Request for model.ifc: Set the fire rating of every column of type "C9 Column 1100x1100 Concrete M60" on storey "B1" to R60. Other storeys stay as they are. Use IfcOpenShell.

First a look at what the model holds.

```python
import ifcopenshell
import ifcopenshell.util.element

model = ifcopenshell.open("model.ifc")
print(model.schema)
storey = next(s for s in model.by_type("IfcBuildingStorey") if s.Name == "B1")
columns = [e for e in ifcopenshell.util.element.get_decomposition(storey) if e.is_a("IfcColumn")]
seen = {}
for e in columns:
    element_type = ifcopenshell.util.element.get_type(e)
    key = (element_type.Name if element_type != e and element_type else None, ifcopenshell.util.element.get_pset(e, "Pset_ColumnCommon", "FireRating"))
    seen[key] = seen.get(key, 0) + 1
for (name, value), count in sorted(seen.items(), key=str):
    print(count, "x", name, "|", value)
```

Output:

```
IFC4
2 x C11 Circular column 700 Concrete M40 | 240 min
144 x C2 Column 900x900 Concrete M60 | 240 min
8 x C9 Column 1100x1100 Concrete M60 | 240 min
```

```python
import ifcopenshell
import ifcopenshell.api.pset
import ifcopenshell.util.element

model = ifcopenshell.open("model.ifc")

storey = next(s for s in model.by_type("IfcBuildingStorey") if s.Name == "B1")
columns = [e for e in ifcopenshell.util.element.get_decomposition(storey) if e.is_a("IfcColumn")]

count = 0
for e in columns:
    element_type = ifcopenshell.util.element.get_type(e)
    if element_type in (None, e) or element_type.Name != "C9 Column 1100x1100 Concrete M60":
        continue
    # add_pset returns the element's existing set when there is one.
    pset = ifcopenshell.api.pset.add_pset(model, product=e, name="Pset_ColumnCommon")
    ifcopenshell.api.pset.edit_pset(model, pset=pset, properties={"FireRating": "R60"})
    count += 1

print(count, "columns updated")

model.write("model-out.ifc")
```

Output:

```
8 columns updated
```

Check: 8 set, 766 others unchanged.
